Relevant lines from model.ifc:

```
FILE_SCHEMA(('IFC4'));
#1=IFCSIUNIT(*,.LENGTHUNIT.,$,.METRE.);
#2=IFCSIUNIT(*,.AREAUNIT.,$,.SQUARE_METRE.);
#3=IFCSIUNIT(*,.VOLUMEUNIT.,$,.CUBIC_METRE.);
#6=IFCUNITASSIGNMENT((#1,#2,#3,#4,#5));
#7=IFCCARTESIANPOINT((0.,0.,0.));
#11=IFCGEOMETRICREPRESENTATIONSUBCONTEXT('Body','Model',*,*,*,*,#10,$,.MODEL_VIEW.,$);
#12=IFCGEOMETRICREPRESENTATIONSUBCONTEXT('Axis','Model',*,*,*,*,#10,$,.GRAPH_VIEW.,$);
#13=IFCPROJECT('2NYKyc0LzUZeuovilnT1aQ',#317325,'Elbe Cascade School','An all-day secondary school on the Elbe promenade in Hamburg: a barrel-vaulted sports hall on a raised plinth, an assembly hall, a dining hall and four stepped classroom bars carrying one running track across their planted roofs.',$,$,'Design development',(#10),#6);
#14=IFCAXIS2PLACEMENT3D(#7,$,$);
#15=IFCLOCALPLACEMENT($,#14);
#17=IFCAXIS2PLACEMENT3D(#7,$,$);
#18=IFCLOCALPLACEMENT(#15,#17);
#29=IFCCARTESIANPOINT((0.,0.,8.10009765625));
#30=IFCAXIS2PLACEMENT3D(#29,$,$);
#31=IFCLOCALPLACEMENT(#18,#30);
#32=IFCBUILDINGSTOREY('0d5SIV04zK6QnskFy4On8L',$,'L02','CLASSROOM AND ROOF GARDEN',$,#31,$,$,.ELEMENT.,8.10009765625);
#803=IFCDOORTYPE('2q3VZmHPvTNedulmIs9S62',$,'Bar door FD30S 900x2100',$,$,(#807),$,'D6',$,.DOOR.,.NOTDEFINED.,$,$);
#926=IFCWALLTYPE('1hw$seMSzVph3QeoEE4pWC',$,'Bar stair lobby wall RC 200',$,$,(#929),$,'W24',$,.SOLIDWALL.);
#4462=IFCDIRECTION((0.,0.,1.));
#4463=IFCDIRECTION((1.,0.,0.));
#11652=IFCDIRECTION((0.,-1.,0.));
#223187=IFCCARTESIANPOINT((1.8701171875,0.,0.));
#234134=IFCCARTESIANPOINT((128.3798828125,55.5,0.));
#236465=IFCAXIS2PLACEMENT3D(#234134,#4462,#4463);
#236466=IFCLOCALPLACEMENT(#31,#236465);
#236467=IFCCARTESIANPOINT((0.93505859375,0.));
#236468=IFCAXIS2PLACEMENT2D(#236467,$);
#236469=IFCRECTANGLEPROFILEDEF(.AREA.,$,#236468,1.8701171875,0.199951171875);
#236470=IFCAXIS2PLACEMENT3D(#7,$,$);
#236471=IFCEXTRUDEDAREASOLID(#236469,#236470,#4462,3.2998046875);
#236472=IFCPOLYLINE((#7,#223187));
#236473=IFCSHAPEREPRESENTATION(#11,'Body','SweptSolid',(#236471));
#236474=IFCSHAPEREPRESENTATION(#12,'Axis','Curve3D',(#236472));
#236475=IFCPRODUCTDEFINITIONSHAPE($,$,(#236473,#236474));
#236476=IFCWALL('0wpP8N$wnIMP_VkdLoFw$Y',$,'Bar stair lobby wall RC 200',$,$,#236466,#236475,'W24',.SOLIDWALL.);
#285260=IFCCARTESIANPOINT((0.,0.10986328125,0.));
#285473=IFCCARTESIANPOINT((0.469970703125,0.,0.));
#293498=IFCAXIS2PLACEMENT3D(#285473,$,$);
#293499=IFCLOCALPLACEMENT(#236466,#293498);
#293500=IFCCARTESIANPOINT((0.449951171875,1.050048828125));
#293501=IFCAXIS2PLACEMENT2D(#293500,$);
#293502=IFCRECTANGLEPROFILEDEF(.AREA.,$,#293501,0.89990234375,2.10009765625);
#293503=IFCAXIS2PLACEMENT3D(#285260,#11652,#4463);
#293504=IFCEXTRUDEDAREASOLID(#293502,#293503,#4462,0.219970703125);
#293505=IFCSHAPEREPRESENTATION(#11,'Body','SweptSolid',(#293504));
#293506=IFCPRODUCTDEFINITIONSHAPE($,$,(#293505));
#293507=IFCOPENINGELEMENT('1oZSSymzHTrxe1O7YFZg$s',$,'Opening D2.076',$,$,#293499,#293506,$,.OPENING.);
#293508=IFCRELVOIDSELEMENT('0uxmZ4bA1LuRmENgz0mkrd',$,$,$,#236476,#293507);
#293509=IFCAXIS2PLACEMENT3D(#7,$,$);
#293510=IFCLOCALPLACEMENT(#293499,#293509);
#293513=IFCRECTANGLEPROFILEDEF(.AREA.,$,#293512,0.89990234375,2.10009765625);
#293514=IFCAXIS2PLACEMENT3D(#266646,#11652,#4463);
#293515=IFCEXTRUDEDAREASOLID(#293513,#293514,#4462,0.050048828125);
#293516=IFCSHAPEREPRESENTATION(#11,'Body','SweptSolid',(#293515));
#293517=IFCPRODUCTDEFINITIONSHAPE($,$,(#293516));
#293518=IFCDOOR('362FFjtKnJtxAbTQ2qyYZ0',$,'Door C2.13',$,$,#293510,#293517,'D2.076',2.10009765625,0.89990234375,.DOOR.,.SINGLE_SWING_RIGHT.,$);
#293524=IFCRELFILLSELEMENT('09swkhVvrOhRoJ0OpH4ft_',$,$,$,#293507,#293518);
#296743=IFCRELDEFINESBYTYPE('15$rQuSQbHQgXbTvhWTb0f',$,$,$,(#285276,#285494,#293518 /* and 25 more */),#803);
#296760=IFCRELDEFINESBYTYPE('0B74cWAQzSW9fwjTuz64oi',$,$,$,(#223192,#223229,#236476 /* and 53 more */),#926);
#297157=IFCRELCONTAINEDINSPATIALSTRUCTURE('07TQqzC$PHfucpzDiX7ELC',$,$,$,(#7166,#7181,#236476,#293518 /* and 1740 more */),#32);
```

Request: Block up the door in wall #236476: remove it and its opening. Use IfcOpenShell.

```python
import ifcopenshell
import ifcopenshell.api.feature
import ifcopenshell.api.root
import ifcopenshell.geom
import ifcopenshell.util.shape

model = ifcopenshell.open("model.ifc")
settings = ifcopenshell.geom.settings()


def volume(element):
    """Net volume in cubic metres, openings subtracted."""
    shape = ifcopenshell.geom.create_shape(settings, element)
    return ifcopenshell.util.shape.get_volume(shape.geometry)


door = model.by_id(293518)
opening = door.FillsVoids[0].RelatingOpeningElement
wall = opening.VoidsElements[0].RelatingBuildingElement
before = volume(wall)

ifcopenshell.api.root.remove_product(model, product=door)
ifcopenshell.api.feature.remove_feature(model, feature=opening)

after = volume(wall)

print(f"wall volume {before:.3f} -> {after:.3f} m3")

model.write("model_updated.ifc")
```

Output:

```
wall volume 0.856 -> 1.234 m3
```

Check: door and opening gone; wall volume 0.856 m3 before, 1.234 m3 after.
